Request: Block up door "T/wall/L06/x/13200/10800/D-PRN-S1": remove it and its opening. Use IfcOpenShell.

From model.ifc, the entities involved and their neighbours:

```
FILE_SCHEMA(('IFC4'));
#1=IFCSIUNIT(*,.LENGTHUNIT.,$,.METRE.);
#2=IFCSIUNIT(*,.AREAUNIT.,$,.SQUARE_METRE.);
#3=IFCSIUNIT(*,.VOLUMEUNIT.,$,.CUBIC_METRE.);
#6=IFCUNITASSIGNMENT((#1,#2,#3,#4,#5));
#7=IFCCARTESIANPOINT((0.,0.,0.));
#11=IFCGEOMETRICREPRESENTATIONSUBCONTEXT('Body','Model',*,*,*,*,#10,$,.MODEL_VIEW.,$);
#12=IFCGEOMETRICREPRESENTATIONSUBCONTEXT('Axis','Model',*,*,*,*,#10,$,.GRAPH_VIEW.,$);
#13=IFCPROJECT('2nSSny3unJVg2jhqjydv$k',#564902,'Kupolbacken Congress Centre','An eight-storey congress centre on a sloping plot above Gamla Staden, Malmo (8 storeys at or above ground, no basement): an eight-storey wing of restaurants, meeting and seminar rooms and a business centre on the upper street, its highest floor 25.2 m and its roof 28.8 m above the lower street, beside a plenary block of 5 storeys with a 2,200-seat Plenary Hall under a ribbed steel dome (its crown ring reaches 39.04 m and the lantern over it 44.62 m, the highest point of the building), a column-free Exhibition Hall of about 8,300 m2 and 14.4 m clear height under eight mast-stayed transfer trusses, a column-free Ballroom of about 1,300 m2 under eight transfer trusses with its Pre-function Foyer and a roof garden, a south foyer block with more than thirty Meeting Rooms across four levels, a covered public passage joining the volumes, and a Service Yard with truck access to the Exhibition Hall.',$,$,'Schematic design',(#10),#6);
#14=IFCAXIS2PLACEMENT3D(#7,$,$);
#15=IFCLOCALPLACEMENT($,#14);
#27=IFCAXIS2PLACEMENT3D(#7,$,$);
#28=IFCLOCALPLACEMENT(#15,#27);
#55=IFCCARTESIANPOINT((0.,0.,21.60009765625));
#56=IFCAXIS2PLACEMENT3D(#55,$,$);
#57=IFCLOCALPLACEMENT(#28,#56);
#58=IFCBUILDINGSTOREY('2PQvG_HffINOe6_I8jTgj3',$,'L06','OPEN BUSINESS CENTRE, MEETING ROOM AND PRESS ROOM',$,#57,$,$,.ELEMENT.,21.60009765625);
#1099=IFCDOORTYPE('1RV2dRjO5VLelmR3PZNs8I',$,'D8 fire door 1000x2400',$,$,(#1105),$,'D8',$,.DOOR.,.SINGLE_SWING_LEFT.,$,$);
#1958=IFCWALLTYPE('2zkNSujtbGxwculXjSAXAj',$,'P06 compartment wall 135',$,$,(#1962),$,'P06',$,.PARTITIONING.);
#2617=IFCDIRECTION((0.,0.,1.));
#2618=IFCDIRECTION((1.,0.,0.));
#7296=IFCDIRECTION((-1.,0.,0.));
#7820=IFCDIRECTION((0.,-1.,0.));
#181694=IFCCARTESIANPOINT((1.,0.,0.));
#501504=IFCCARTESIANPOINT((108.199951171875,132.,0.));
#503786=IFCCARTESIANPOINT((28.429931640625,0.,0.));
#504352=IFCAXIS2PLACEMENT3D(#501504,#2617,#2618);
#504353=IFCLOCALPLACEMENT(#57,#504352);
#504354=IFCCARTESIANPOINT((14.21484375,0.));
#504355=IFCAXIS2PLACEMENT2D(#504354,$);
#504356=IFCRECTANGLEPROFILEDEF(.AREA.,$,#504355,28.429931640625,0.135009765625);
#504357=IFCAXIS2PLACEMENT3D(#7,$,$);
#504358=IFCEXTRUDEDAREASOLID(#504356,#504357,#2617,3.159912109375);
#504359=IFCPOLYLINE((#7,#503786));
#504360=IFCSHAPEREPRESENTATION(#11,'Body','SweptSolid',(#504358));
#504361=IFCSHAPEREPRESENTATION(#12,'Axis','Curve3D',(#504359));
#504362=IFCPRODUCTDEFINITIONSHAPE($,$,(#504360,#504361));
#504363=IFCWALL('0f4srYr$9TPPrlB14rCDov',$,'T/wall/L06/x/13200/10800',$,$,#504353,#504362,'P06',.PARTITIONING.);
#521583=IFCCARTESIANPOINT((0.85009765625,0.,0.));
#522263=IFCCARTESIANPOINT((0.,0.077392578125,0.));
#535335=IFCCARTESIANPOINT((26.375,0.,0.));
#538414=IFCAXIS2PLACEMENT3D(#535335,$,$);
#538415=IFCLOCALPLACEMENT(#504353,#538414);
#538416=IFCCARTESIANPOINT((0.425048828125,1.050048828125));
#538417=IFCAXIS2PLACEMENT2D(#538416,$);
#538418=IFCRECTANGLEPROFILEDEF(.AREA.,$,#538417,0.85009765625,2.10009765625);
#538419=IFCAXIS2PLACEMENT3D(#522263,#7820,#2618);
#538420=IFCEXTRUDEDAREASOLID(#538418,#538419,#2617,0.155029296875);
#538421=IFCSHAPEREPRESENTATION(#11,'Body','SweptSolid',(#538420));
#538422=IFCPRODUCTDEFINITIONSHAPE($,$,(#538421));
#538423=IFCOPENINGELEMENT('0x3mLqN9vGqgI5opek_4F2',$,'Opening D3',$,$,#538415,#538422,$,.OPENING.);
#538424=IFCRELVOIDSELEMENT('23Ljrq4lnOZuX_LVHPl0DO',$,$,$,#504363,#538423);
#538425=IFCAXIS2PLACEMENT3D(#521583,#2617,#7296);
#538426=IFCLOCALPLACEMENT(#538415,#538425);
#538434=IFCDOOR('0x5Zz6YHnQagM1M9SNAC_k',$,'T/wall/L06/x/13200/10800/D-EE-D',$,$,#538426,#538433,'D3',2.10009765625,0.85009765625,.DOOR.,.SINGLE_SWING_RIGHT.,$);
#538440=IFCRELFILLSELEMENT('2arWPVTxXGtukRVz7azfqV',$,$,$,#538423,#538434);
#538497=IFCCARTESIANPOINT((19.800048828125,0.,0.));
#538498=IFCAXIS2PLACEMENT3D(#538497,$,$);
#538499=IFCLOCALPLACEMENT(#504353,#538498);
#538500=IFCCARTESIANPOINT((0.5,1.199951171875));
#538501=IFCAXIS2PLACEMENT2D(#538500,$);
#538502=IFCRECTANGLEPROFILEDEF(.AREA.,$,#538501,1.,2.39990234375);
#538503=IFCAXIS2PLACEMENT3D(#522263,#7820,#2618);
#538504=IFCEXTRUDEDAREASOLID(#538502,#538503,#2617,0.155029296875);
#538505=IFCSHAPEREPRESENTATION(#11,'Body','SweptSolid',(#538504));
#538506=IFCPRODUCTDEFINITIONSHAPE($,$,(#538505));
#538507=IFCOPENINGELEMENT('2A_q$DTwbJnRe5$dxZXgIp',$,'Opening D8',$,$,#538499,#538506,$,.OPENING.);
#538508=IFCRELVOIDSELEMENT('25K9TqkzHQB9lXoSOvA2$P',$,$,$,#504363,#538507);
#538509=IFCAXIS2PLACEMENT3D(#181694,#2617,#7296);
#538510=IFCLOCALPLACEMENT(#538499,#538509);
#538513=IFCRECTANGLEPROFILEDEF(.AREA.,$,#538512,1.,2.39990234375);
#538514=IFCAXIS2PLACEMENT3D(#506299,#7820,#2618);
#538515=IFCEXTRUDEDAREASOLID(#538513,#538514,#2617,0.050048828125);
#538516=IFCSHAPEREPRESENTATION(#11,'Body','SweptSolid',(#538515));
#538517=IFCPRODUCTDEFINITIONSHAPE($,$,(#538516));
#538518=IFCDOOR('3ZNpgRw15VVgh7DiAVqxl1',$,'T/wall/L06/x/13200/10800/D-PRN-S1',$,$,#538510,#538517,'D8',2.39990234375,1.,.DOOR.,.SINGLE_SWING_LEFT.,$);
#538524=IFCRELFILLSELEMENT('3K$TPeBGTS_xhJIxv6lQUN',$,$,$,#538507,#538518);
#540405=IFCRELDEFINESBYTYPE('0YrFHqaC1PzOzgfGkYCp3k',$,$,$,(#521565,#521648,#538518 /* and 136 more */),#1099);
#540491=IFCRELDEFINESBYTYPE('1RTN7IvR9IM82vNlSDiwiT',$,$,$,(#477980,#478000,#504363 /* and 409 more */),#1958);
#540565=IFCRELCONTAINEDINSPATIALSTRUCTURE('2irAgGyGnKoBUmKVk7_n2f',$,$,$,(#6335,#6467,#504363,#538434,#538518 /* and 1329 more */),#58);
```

```python
import ifcopenshell
import ifcopenshell.api.feature
import ifcopenshell.api.root
import ifcopenshell.geom
import ifcopenshell.util.shape

model = ifcopenshell.open("model.ifc")
settings = ifcopenshell.geom.settings()


def volume(element):
    """Net volume in cubic metres, openings subtracted."""
    shape = ifcopenshell.geom.create_shape(settings, element)
    return ifcopenshell.util.shape.get_volume(shape.geometry)


door = model.by_id(538518)
opening = door.FillsVoids[0].RelatingOpeningElement
wall = opening.VoidsElements[0].RelatingBuildingElement
before = volume(wall)

ifcopenshell.api.root.remove_product(model, product=door)
ifcopenshell.api.feature.remove_feature(model, feature=opening)

after = volume(wall)

print(f"wall volume {before:.3f} -> {after:.3f} m3")

model.write("model_rev.ifc")
```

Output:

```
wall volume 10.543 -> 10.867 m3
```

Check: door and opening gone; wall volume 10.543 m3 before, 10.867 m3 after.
